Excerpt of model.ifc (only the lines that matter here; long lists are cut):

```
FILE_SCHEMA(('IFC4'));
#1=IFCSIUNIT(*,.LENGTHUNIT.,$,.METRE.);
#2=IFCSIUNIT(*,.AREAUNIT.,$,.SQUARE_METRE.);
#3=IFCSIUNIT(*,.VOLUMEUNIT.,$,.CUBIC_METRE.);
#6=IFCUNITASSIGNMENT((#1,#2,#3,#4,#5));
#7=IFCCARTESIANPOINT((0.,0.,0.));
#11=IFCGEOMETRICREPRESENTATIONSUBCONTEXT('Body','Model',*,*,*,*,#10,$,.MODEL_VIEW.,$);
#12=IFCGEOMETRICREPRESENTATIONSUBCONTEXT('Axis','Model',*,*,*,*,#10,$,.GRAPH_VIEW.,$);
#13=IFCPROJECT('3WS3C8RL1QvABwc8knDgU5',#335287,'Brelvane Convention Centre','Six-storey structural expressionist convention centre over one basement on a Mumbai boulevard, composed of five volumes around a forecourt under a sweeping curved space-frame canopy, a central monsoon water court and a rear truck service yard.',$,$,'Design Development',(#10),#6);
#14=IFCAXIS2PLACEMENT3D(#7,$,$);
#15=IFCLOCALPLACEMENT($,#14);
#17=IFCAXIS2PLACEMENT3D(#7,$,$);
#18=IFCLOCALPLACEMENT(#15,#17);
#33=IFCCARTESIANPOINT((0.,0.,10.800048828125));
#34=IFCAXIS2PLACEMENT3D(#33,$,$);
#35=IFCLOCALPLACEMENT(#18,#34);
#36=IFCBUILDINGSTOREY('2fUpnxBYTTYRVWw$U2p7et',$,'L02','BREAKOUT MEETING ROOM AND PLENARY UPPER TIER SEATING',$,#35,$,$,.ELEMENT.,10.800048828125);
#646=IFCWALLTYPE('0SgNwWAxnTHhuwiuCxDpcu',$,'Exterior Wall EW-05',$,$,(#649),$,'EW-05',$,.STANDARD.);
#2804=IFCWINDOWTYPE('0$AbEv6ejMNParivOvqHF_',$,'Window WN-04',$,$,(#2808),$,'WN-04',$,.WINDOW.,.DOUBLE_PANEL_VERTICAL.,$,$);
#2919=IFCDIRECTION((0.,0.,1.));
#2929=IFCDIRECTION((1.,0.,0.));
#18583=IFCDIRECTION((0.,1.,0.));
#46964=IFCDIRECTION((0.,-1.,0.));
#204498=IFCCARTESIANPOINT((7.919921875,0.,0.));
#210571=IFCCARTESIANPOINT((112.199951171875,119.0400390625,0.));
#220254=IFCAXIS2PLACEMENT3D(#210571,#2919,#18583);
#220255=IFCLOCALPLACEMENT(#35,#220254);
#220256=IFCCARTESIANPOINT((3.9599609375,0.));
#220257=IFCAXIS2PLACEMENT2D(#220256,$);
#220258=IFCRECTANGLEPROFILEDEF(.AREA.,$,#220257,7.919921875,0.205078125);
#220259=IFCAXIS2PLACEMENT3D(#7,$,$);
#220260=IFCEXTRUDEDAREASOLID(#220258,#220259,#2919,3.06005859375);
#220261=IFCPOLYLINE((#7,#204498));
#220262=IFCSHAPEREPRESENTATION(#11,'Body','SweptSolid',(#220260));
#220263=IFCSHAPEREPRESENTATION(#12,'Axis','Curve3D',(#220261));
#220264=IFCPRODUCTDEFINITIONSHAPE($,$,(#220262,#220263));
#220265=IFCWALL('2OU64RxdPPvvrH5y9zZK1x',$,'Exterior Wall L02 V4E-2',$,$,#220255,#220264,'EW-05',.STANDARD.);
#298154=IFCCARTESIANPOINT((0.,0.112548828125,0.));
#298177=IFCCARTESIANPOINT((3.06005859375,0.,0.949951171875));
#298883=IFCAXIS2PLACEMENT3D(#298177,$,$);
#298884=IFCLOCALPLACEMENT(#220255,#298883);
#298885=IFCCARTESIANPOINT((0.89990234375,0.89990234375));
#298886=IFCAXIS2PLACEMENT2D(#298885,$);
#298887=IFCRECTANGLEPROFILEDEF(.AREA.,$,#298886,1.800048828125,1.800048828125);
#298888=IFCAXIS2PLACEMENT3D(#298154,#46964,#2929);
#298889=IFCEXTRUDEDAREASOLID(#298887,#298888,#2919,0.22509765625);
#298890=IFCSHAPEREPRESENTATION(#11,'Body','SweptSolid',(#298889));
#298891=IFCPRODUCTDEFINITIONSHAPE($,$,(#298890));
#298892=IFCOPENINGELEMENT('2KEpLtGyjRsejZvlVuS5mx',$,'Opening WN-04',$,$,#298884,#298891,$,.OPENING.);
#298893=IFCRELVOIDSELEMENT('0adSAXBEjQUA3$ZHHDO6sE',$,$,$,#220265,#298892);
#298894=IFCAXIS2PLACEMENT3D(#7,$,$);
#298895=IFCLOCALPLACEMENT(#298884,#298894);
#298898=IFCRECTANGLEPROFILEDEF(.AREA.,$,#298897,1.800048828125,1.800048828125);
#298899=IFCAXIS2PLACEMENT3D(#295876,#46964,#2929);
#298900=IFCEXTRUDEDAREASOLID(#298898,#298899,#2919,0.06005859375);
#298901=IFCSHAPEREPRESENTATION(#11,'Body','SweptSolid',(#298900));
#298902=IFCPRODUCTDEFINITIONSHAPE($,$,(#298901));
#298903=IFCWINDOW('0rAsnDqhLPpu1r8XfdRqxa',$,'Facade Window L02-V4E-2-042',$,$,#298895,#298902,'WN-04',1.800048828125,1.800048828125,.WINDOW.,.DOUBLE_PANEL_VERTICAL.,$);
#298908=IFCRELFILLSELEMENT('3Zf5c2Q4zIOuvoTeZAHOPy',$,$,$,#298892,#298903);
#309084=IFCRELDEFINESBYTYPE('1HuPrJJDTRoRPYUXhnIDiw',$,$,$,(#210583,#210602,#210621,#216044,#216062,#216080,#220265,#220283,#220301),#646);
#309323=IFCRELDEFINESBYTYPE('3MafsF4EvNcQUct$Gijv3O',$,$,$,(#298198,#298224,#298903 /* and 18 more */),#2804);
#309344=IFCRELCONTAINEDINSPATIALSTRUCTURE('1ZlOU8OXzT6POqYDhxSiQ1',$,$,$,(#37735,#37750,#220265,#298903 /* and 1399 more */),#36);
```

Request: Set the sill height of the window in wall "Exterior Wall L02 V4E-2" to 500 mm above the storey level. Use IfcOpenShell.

```python
import numpy as np
import ifcopenshell
import ifcopenshell.api.geometry
import ifcopenshell.geom
import ifcopenshell.util.element
import ifcopenshell.util.placement
import ifcopenshell.util.shape
import ifcopenshell.util.unit

model = ifcopenshell.open("model.ifc")
unit_scale = ifcopenshell.util.unit.calculate_unit_scale(model)

window = model.by_id(298903)
opening = window.FillsVoids[0].RelatingOpeningElement
storey = ifcopenshell.util.element.get_container(window, ifc_class="IfcBuildingStorey")
level = ifcopenshell.util.placement.get_local_placement(storey.ObjectPlacement)[2, 3]

# The opening's origin need not be at the sill, so measure its lowest point.
shape = ifcopenshell.geom.create_shape(ifcopenshell.geom.settings(), opening)
bottom = ifcopenshell.util.shape.get_shape_bottom_elevation(shape, shape.geometry) / unit_scale
dz = level + 0.5 / unit_scale - bottom

shift = np.array([0.0, 0.0, dz])
# The window is placed relative to its opening, so it follows when the opening moves.
matrix = ifcopenshell.util.placement.get_local_placement(opening.ObjectPlacement)
matrix[:3, 3] += shift
ifcopenshell.api.geometry.edit_object_placement(
    model, product=opening, matrix=matrix, is_si=False, should_transform_children=True
)

print(f"moved by {dz * unit_scale:+.3f} m")

model.write("model_rev.ifc")
```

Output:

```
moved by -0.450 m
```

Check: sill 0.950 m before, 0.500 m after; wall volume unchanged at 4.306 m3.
